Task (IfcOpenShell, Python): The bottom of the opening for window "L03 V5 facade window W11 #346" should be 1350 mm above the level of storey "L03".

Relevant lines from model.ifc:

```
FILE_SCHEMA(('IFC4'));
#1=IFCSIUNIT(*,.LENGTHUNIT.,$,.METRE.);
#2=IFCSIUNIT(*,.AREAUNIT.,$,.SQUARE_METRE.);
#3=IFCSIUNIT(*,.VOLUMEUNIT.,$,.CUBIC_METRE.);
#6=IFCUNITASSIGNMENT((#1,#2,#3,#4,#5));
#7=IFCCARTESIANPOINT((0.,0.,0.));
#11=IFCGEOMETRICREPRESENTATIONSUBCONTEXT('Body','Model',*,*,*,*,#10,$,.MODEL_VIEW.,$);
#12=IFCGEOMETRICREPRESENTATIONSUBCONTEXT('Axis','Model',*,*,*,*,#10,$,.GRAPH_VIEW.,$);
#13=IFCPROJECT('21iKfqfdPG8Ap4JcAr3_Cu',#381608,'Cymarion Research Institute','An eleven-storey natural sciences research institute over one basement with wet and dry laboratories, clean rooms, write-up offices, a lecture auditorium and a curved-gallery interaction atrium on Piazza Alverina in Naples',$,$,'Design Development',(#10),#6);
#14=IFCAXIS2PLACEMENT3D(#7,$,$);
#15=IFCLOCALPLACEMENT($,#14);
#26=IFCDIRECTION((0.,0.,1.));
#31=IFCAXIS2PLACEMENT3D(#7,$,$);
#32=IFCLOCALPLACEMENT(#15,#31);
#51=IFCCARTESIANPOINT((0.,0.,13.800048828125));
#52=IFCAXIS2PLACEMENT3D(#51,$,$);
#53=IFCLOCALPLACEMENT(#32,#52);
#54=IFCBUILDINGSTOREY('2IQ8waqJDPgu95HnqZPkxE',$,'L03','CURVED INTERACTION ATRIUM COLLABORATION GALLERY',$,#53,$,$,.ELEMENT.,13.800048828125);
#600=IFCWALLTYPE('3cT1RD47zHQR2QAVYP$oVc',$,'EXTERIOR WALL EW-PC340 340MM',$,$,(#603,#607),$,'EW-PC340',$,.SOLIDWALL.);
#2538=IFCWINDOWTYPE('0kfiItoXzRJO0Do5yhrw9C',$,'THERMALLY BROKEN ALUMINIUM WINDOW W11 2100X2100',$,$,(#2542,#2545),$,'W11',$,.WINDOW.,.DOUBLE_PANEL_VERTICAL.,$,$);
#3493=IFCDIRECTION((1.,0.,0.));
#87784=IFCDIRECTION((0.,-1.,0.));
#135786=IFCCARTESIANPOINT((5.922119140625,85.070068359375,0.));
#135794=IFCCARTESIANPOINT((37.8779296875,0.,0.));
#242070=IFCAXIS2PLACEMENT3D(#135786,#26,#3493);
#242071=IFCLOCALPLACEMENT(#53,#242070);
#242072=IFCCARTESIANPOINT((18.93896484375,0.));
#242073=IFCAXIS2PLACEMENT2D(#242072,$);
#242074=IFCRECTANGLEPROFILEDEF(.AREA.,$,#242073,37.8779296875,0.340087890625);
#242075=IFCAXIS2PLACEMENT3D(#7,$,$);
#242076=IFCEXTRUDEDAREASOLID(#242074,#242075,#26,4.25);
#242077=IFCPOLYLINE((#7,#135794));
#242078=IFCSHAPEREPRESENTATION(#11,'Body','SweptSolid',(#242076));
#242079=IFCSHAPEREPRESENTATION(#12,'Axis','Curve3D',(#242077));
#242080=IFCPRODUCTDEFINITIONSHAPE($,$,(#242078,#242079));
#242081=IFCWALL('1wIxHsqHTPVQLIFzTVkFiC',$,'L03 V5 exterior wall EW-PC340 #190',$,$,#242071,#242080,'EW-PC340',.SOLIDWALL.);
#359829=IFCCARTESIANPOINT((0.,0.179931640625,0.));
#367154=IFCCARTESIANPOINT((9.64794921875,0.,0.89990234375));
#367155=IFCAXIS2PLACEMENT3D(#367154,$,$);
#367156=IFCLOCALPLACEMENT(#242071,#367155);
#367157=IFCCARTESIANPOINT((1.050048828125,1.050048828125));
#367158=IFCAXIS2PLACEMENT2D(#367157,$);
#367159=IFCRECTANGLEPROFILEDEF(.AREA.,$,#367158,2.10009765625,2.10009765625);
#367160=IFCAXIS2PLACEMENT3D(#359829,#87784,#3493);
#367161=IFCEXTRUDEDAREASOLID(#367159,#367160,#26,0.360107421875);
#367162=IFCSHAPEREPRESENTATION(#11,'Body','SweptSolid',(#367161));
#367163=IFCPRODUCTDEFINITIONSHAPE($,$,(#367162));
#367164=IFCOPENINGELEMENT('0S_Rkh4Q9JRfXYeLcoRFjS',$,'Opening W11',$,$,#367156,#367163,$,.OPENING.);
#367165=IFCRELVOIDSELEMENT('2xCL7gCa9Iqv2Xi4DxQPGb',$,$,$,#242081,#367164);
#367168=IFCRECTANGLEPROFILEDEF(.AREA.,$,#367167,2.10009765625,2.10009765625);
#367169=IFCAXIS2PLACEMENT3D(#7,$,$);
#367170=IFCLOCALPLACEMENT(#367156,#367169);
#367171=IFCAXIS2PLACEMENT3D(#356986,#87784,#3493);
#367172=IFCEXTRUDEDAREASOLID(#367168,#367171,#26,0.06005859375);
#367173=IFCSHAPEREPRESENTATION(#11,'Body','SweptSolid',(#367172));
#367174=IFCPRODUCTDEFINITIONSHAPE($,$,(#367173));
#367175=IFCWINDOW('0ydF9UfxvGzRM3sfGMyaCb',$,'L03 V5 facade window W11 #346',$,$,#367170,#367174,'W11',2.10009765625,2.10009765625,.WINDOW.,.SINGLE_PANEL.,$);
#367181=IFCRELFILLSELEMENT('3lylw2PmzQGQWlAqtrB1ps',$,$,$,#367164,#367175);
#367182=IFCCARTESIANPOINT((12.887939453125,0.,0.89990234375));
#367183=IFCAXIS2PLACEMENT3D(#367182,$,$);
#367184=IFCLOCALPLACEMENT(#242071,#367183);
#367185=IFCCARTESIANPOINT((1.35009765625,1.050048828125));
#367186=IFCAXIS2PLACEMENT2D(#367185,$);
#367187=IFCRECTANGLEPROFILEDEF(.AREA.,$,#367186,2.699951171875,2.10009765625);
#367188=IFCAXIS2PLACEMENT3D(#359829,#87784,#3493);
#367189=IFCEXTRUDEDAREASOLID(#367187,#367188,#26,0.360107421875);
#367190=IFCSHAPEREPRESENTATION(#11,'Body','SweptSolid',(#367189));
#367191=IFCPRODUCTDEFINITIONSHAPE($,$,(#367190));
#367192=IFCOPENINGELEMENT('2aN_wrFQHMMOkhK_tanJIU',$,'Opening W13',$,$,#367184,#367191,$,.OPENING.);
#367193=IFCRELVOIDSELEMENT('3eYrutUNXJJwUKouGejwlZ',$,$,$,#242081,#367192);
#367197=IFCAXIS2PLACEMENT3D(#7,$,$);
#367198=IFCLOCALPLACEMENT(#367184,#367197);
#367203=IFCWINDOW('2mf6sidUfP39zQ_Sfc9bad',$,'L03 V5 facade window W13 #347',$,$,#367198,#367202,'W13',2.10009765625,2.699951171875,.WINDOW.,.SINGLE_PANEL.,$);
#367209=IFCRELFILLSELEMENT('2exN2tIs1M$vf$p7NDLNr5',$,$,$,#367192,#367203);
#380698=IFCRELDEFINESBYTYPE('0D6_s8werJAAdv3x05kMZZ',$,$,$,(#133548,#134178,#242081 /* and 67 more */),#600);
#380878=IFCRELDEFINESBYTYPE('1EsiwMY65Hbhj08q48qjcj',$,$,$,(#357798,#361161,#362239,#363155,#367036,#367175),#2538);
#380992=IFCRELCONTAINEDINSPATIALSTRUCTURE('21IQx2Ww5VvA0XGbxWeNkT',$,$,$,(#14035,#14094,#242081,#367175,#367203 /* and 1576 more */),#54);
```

```python
import numpy as np
import ifcopenshell
import ifcopenshell.api.geometry
import ifcopenshell.geom
import ifcopenshell.util.element
import ifcopenshell.util.placement
import ifcopenshell.util.shape
import ifcopenshell.util.unit

model = ifcopenshell.open("model.ifc")
unit_scale = ifcopenshell.util.unit.calculate_unit_scale(model)

window = model.by_guid("0ydF9UfxvGzRM3sfGMyaCb")
opening = window.FillsVoids[0].RelatingOpeningElement
storey = ifcopenshell.util.element.get_container(window, ifc_class="IfcBuildingStorey")
level = ifcopenshell.util.placement.get_local_placement(storey.ObjectPlacement)[2, 3]

# The opening's origin need not be at the sill, so measure its lowest point.
shape = ifcopenshell.geom.create_shape(ifcopenshell.geom.settings(), opening)
bottom = ifcopenshell.util.shape.get_shape_bottom_elevation(shape, shape.geometry) / unit_scale
dz = level + 1.35 - bottom

shift = np.array([0.0, 0.0, dz])
# The window is placed relative to its opening, so it follows when the opening moves.
matrix = ifcopenshell.util.placement.get_local_placement(opening.ObjectPlacement)
matrix[:3, 3] += shift
ifcopenshell.api.geometry.edit_object_placement(
    model, product=opening, matrix=matrix, is_si=False, should_transform_children=True
)

print(f"moved by {dz * unit_scale:+.3f} m")

model.write("model_rev.ifc")
```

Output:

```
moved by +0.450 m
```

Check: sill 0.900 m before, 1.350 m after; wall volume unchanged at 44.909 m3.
